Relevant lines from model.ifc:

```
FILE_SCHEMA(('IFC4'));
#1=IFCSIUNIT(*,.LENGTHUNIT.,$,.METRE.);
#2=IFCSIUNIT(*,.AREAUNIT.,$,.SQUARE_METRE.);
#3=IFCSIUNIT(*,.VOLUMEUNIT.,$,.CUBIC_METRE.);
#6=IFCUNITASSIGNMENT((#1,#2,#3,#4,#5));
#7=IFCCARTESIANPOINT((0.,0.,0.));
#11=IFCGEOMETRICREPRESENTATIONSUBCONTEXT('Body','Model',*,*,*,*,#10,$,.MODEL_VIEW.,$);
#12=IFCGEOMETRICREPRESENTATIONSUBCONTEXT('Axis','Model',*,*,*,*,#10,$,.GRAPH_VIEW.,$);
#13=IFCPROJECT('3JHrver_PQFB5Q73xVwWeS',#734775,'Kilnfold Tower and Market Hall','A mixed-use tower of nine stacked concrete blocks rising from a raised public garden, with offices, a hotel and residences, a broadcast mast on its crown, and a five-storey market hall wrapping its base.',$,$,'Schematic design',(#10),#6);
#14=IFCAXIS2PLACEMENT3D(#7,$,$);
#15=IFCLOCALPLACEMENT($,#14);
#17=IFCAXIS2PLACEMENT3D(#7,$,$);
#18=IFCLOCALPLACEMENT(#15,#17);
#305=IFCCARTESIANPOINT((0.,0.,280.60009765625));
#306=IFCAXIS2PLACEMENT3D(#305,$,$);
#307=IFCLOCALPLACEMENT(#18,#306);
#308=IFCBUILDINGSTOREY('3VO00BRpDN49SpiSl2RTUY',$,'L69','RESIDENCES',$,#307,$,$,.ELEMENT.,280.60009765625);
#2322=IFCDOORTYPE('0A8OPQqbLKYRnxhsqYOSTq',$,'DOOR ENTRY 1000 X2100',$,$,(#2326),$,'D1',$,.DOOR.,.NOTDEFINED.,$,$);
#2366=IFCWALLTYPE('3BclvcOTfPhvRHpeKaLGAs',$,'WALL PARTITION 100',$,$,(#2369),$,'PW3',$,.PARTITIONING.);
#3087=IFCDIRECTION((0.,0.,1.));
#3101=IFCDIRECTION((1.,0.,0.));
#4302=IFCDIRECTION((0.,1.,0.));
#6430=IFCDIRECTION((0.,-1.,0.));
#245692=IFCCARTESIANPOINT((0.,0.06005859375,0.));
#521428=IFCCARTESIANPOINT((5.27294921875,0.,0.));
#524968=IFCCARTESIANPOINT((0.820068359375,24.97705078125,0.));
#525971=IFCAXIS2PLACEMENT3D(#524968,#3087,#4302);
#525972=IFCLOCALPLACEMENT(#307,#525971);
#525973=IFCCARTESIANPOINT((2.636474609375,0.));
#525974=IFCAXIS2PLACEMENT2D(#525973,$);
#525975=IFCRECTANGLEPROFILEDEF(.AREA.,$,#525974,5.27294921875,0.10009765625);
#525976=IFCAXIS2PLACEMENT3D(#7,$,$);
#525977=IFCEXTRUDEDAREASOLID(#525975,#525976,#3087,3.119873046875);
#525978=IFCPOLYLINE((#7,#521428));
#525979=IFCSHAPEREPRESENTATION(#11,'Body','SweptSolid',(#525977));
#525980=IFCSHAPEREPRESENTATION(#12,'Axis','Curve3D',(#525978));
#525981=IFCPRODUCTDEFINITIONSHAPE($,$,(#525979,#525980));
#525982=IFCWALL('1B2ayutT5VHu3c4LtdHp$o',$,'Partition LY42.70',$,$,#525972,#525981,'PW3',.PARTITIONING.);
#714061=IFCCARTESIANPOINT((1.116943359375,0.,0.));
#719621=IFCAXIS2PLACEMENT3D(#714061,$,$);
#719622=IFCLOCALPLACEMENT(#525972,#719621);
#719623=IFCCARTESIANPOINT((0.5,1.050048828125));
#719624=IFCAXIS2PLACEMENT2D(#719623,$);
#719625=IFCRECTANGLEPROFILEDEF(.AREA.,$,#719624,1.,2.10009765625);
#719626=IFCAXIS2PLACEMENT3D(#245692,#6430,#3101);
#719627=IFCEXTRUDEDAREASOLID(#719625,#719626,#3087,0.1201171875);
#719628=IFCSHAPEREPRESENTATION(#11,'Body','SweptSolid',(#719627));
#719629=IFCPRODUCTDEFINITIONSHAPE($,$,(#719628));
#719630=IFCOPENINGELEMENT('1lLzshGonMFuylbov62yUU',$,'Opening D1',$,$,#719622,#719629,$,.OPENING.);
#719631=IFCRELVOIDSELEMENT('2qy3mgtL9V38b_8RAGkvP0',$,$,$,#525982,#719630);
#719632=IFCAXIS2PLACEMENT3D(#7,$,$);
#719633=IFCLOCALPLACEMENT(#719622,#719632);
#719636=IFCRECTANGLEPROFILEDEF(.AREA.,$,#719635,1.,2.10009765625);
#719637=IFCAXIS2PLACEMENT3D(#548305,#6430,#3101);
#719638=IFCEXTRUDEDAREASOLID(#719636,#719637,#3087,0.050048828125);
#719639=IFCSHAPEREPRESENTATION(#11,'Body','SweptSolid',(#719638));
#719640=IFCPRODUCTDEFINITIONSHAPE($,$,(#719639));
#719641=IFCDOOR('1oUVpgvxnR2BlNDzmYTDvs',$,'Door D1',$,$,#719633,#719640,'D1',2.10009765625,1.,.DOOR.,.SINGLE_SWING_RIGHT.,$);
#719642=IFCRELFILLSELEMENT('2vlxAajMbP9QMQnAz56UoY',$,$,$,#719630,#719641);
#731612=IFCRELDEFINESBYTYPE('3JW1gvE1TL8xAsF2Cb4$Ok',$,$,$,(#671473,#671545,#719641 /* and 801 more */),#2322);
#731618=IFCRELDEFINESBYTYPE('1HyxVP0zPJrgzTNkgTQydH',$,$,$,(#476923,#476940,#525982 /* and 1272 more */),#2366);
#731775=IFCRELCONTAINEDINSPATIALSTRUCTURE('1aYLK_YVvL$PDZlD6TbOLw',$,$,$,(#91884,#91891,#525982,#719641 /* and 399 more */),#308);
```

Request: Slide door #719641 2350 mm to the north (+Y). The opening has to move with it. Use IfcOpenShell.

```python
import ifcopenshell
import ifcopenshell.api.geometry
import ifcopenshell.util.placement

model = ifcopenshell.open("model.ifc")

door = model.by_id(719641)
opening = door.FillsVoids[0].RelatingOpeningElement
wall = opening.VoidsElements[0].RelatingBuildingElement

wall_matrix = ifcopenshell.util.placement.get_local_placement(wall.ObjectPlacement)
shift = wall_matrix[:3, 0] * 2.35
before = ifcopenshell.util.placement.get_local_placement(door.ObjectPlacement)[:3, 3].copy()

# The door is placed relative to its opening, so it follows when the opening moves.
matrix = ifcopenshell.util.placement.get_local_placement(opening.ObjectPlacement)
matrix[:3, 3] += shift
ifcopenshell.api.geometry.edit_object_placement(
    model, product=opening, matrix=matrix, is_si=False, should_transform_children=True
)

after = ifcopenshell.util.placement.get_local_placement(door.ObjectPlacement)[:3, 3]
print("door moved by", (after - before).round(3) + 0.0)

model.write("model_updated.ifc")
```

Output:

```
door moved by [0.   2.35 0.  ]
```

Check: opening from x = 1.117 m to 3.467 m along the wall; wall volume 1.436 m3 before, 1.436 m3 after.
